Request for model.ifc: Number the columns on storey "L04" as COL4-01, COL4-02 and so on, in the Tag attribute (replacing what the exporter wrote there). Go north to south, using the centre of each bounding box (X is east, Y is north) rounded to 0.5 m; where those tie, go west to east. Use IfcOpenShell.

First a look at what the model holds.

```python
import ifcopenshell
import ifcopenshell.util.element
import ifcopenshell.util.placement

model = ifcopenshell.open("model.ifc")
print(model.schema)
storey = next(s for s in model.by_type("IfcBuildingStorey") if s.Name == "L04")
columns = [e for e in ifcopenshell.util.element.get_decomposition(storey) if e.is_a("IfcColumn")]
for e in sorted(columns, key=lambda e: e.id()):
    origin = ifcopenshell.util.placement.get_local_placement(e.ObjectPlacement)[:3, 3]
    print(e.id(), e.Tag, e.Name, origin.round(2) + 0.0, sep=" | ")
```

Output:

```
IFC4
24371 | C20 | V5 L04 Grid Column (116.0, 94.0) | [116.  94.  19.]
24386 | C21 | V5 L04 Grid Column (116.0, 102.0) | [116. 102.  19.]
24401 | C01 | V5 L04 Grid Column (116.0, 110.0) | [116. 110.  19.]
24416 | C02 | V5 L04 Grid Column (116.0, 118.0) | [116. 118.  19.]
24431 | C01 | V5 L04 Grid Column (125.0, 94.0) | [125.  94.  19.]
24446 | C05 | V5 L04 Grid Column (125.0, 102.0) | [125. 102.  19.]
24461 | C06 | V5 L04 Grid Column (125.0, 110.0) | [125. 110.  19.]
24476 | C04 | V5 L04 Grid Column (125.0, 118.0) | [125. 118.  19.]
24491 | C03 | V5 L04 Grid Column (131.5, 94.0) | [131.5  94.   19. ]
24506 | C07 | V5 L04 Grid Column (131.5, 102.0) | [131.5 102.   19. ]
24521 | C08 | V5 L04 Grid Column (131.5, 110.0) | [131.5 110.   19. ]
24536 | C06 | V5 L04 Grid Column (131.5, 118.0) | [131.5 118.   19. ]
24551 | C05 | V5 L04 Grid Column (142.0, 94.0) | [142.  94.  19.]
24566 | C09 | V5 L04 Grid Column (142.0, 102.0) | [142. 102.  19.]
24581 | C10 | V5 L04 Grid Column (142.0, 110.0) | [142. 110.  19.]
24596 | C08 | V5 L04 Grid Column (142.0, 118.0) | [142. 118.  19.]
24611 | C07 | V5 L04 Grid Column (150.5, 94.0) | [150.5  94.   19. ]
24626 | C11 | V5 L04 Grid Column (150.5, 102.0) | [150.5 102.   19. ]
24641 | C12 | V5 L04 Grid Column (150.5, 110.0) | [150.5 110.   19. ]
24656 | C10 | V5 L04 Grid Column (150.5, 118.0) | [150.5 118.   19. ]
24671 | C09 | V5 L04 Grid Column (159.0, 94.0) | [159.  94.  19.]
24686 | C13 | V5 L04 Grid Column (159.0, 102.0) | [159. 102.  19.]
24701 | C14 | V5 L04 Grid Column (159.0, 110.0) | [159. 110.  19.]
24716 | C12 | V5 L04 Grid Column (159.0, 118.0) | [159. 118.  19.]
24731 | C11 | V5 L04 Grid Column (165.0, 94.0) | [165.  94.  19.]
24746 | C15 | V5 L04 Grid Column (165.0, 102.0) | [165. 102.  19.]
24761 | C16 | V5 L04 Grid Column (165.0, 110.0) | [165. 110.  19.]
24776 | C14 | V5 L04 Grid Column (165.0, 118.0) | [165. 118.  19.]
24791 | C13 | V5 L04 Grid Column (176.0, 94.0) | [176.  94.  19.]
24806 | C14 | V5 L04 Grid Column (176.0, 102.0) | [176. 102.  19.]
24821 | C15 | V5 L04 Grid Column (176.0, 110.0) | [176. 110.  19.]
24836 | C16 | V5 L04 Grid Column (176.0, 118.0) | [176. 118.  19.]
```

```python
import ifcopenshell
import ifcopenshell.geom
import ifcopenshell.util.element
import ifcopenshell.util.shape

model = ifcopenshell.open("model.ifc")
settings = ifcopenshell.geom.settings()
settings.set("use-world-coords", True)


def centre(element):
    shape = ifcopenshell.geom.create_shape(settings, element)
    return ifcopenshell.util.shape.get_bbox_centroid(shape.geometry)


storey = next(s for s in model.by_type("IfcBuildingStorey") if s.Name == "L04")
columns = [e for e in ifcopenshell.util.element.get_decomposition(storey) if e.is_a("IfcColumn")]

# Insertion points can sit at a corner or the storey origin, so sort by the geometry (in metres).
centres = {e: centre(e) for e in columns}
columns.sort(key=lambda e: (-round(centres[e][1] / 0.5), centres[e][0]))

for i, e in enumerate(columns, start=1):
    number = f"COL4-{i:02d}"
    e.Tag = number
    print(e.id(), number)

model.write("model-out.ifc")
```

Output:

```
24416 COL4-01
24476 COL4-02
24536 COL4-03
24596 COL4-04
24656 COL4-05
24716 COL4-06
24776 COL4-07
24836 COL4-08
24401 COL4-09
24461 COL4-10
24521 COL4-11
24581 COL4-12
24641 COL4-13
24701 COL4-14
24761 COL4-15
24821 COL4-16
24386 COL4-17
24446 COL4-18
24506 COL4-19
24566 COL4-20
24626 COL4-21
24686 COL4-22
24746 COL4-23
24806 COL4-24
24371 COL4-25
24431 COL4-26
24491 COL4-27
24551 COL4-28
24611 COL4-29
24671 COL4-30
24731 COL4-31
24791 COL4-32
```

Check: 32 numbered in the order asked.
